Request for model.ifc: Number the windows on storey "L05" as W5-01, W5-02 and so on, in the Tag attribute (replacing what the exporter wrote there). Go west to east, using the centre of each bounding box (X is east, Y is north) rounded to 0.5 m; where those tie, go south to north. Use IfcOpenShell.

First a look at what the model holds.

```python
import ifcopenshell
import ifcopenshell.util.element
import ifcopenshell.util.placement

model = ifcopenshell.open("model.ifc")
print(model.schema)
storey = next(s for s in model.by_type("IfcBuildingStorey") if s.Name == "L05")
windows = [e for e in ifcopenshell.util.element.get_decomposition(storey) if e.is_a("IfcWindow")]
for e in sorted(windows, key=lambda e: e.id()):
    origin = ifcopenshell.util.placement.get_local_placement(e.ObjectPlacement)[:3, 3]
    print(e.id(), e.Tag, e.Name, origin.round(2) + 0.0, sep=" | ")
```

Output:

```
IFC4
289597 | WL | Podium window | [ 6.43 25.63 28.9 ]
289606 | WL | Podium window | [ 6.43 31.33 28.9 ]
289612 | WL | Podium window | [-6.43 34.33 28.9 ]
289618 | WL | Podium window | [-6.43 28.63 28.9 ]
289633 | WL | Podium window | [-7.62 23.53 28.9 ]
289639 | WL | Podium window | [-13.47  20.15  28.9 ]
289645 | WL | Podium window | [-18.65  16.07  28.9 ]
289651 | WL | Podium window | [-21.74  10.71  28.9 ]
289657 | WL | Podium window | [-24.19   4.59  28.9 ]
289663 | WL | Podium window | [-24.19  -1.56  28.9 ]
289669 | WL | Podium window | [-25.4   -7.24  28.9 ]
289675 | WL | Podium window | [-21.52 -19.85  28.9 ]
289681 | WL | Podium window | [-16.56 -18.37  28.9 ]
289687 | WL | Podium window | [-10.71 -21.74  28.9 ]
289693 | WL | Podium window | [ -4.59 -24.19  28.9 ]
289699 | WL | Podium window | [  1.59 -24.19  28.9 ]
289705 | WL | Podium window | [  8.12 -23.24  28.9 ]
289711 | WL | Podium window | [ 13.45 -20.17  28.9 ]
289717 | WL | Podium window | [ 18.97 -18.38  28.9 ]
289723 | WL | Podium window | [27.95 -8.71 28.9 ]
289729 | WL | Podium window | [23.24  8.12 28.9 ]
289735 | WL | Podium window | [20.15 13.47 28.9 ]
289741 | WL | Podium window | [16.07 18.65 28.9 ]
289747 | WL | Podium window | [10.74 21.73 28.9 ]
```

```python
import ifcopenshell
import ifcopenshell.geom
import ifcopenshell.util.element
import ifcopenshell.util.shape

model = ifcopenshell.open("model.ifc")
settings = ifcopenshell.geom.settings()
settings.set("use-world-coords", True)


def centre(element):
    shape = ifcopenshell.geom.create_shape(settings, element)
    return ifcopenshell.util.shape.get_bbox_centroid(shape.geometry)


storey = next(s for s in model.by_type("IfcBuildingStorey") if s.Name == "L05")
windows = [e for e in ifcopenshell.util.element.get_decomposition(storey) if e.is_a("IfcWindow")]

# Insertion points can sit at a corner or the storey origin, so sort by the geometry (in metres).
centres = {e: centre(e) for e in windows}
windows.sort(key=lambda e: (round(centres[e][0] / 0.5), centres[e][1]))

for i, e in enumerate(windows, start=1):
    number = f"W5-{i:02d}"
    e.Tag = number
    print(e.id(), number)

model.write("model-out.ifc")
```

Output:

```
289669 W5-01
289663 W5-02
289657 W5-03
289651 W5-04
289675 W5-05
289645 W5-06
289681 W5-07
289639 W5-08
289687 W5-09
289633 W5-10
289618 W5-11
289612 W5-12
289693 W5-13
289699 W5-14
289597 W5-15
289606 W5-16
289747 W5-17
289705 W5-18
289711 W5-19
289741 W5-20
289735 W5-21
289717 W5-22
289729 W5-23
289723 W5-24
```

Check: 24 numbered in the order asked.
